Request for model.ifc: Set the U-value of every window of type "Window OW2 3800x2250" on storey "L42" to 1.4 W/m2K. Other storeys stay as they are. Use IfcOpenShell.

First a look at what the model holds.

```python
import ifcopenshell
import ifcopenshell.util.element

model = ifcopenshell.open("model.ifc")
print(model.schema)
storey = next(s for s in model.by_type("IfcBuildingStorey") if s.Name == "L42")
windows = [e for e in ifcopenshell.util.element.get_decomposition(storey) if e.is_a("IfcWindow")]
seen = {}
for e in windows:
    element_type = ifcopenshell.util.element.get_type(e)
    key = (element_type.Name if element_type != e and element_type else None, ifcopenshell.util.element.get_pset(e, "Pset_WindowCommon", "ThermalTransmittance"))
    seen[key] = seen.get(key, 0) + 1
for (name, value), count in sorted(seen.items(), key=str):
    print(count, "x", name, "|", value)
```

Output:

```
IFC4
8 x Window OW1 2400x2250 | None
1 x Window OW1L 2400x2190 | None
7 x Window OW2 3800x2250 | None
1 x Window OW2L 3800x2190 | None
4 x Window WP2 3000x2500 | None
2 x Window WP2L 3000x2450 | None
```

```python
import ifcopenshell
import ifcopenshell.api.pset
import ifcopenshell.util.element

model = ifcopenshell.open("model.ifc")

storey = next(s for s in model.by_type("IfcBuildingStorey") if s.Name == "L42")
windows = [e for e in ifcopenshell.util.element.get_decomposition(storey) if e.is_a("IfcWindow")]

count = 0
for e in windows:
    element_type = ifcopenshell.util.element.get_type(e)
    if element_type in (None, e) or element_type.Name != "Window OW2 3800x2250":
        continue
    found = ifcopenshell.util.element.get_pset(e, "Pset_WindowCommon", should_inherit=False)
    if found:
        pset = model.by_id(found["id"])
        if len(ifcopenshell.util.element.get_elements_by_pset(pset)) > 1:
            pset = ifcopenshell.api.pset.unshare_pset(model, products=[e], pset=pset)[0]
    else:
        pset = ifcopenshell.api.pset.add_pset(model, product=e, name="Pset_WindowCommon")
    ifcopenshell.api.pset.edit_pset(model, pset=pset, properties={"ThermalTransmittance": 1.4})
    count += 1

print(count, "windows updated")

model.write("model_v2.ifc")
```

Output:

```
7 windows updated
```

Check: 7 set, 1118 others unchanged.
